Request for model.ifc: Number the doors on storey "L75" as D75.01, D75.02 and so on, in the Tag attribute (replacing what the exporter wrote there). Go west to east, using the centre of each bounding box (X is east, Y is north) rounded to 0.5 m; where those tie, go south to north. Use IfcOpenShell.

First a look at what the model holds.

```python
import ifcopenshell
import ifcopenshell.util.element
import ifcopenshell.util.placement

model = ifcopenshell.open("model.ifc")
print(model.schema)
storey = next(s for s in model.by_type("IfcBuildingStorey") if s.Name == "L75")
doors = [e for e in ifcopenshell.util.element.get_decomposition(storey) if e.is_a("IfcDoor")]
for e in sorted(doors, key=lambda e: e.id()):
    origin = ifcopenshell.util.placement.get_local_placement(e.ObjectPlacement)[:3, 3]
    print(e.id(), e.Tag, e.Name, origin.round(2) + 0.0, sep=" | ")
```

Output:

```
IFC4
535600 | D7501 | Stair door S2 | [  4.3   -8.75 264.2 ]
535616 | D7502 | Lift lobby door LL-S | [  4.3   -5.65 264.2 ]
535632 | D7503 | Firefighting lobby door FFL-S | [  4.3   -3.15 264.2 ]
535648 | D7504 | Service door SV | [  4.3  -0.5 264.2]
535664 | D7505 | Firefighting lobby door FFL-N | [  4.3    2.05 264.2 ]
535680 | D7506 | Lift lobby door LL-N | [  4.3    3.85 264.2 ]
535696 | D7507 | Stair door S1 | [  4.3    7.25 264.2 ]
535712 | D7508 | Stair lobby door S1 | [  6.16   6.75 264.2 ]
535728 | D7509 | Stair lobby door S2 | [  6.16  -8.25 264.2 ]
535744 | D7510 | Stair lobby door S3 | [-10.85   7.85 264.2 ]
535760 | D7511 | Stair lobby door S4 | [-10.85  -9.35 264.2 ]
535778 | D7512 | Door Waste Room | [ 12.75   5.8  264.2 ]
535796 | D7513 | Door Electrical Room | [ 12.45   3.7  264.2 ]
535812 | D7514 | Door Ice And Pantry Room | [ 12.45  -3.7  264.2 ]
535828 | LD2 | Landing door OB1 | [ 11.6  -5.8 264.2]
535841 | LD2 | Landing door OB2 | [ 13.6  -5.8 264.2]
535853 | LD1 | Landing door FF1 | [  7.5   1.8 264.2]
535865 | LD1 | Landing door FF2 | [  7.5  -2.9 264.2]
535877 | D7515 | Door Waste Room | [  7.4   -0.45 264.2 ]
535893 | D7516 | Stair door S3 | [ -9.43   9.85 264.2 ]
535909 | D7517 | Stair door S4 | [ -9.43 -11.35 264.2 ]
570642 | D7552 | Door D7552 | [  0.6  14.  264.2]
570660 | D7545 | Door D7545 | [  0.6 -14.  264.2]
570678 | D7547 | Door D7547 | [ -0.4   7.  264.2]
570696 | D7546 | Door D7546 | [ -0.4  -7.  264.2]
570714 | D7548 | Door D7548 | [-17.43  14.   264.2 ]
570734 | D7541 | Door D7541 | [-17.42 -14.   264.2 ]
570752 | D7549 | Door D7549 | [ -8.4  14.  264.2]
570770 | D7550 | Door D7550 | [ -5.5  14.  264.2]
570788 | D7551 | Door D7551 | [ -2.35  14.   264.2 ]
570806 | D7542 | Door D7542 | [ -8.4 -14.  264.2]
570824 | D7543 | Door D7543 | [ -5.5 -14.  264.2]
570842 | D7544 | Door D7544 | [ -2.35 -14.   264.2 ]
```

```python
import ifcopenshell
import ifcopenshell.geom
import ifcopenshell.util.element
import ifcopenshell.util.shape

model = ifcopenshell.open("model.ifc")
settings = ifcopenshell.geom.settings()
settings.set("use-world-coords", True)


def centre(element):
    shape = ifcopenshell.geom.create_shape(settings, element)
    return ifcopenshell.util.shape.get_bbox_centroid(shape.geometry)


storey = next(s for s in model.by_type("IfcBuildingStorey") if s.Name == "L75")
doors = [e for e in ifcopenshell.util.element.get_decomposition(storey) if e.is_a("IfcDoor")]

# Insertion points can sit at a corner or the storey origin, so sort by the geometry (in metres).
centres = {e: centre(e) for e in doors}
doors.sort(key=lambda e: (round(centres[e][0] / 0.5), centres[e][1]))

for i, e in enumerate(doors, start=1):
    number = f"D75.{i:02d}"
    e.Tag = number
    print(e.id(), number)

model.write("model_edited.ifc")
```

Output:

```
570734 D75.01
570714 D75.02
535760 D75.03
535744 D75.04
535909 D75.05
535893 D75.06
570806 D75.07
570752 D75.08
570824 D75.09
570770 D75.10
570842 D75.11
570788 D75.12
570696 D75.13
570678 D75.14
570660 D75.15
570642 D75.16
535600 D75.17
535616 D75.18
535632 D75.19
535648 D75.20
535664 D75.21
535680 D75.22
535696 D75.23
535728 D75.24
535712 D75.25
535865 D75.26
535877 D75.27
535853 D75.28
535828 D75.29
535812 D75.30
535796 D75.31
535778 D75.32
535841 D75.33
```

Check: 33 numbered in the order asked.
